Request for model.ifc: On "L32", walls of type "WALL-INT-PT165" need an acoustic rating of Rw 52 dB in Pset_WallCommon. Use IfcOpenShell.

First a look at what the model holds.

```python
import ifcopenshell
import ifcopenshell.util.element

model = ifcopenshell.open("model.ifc")
print(model.schema)
storey = next(s for s in model.by_type("IfcBuildingStorey") if s.Name == "L32")
walls = [e for e in ifcopenshell.util.element.get_decomposition(storey) if e.is_a("IfcWall")]
seen = {}
for e in walls:
    element_type = ifcopenshell.util.element.get_type(e)
    key = (element_type.Name if element_type != e and element_type else None, ifcopenshell.util.element.get_pset(e, "Pset_WallCommon", "AcousticRating"))
    seen[key] = seen.get(key, 0) + 1
for (name, value), count in sorted(seen.items(), key=str):
    print(count, "x", name, "|", value)
```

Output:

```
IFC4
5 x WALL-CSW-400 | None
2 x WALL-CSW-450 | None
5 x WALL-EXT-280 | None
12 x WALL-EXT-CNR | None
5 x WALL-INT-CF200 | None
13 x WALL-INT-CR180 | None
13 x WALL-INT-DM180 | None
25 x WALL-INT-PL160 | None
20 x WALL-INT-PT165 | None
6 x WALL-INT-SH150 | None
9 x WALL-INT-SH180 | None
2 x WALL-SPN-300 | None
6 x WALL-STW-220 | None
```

```python
import ifcopenshell
import ifcopenshell.api.pset
import ifcopenshell.util.element

model = ifcopenshell.open("model.ifc")

storey = next(s for s in model.by_type("IfcBuildingStorey") if s.Name == "L32")
walls = [e for e in ifcopenshell.util.element.get_decomposition(storey) if e.is_a("IfcWall")]

count = 0
for e in walls:
    element_type = ifcopenshell.util.element.get_type(e)
    if element_type in (None, e) or element_type.Name != "WALL-INT-PT165":
        continue
    # add_pset returns the element's existing set when there is one.
    pset = ifcopenshell.api.pset.add_pset(model, product=e, name="Pset_WallCommon")
    ifcopenshell.api.pset.edit_pset(model, pset=pset, properties={"AcousticRating": "Rw 52 dB"})
    count += 1

print(count, "walls updated")

model.write("model-out.ifc")
```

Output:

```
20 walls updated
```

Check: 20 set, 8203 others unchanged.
